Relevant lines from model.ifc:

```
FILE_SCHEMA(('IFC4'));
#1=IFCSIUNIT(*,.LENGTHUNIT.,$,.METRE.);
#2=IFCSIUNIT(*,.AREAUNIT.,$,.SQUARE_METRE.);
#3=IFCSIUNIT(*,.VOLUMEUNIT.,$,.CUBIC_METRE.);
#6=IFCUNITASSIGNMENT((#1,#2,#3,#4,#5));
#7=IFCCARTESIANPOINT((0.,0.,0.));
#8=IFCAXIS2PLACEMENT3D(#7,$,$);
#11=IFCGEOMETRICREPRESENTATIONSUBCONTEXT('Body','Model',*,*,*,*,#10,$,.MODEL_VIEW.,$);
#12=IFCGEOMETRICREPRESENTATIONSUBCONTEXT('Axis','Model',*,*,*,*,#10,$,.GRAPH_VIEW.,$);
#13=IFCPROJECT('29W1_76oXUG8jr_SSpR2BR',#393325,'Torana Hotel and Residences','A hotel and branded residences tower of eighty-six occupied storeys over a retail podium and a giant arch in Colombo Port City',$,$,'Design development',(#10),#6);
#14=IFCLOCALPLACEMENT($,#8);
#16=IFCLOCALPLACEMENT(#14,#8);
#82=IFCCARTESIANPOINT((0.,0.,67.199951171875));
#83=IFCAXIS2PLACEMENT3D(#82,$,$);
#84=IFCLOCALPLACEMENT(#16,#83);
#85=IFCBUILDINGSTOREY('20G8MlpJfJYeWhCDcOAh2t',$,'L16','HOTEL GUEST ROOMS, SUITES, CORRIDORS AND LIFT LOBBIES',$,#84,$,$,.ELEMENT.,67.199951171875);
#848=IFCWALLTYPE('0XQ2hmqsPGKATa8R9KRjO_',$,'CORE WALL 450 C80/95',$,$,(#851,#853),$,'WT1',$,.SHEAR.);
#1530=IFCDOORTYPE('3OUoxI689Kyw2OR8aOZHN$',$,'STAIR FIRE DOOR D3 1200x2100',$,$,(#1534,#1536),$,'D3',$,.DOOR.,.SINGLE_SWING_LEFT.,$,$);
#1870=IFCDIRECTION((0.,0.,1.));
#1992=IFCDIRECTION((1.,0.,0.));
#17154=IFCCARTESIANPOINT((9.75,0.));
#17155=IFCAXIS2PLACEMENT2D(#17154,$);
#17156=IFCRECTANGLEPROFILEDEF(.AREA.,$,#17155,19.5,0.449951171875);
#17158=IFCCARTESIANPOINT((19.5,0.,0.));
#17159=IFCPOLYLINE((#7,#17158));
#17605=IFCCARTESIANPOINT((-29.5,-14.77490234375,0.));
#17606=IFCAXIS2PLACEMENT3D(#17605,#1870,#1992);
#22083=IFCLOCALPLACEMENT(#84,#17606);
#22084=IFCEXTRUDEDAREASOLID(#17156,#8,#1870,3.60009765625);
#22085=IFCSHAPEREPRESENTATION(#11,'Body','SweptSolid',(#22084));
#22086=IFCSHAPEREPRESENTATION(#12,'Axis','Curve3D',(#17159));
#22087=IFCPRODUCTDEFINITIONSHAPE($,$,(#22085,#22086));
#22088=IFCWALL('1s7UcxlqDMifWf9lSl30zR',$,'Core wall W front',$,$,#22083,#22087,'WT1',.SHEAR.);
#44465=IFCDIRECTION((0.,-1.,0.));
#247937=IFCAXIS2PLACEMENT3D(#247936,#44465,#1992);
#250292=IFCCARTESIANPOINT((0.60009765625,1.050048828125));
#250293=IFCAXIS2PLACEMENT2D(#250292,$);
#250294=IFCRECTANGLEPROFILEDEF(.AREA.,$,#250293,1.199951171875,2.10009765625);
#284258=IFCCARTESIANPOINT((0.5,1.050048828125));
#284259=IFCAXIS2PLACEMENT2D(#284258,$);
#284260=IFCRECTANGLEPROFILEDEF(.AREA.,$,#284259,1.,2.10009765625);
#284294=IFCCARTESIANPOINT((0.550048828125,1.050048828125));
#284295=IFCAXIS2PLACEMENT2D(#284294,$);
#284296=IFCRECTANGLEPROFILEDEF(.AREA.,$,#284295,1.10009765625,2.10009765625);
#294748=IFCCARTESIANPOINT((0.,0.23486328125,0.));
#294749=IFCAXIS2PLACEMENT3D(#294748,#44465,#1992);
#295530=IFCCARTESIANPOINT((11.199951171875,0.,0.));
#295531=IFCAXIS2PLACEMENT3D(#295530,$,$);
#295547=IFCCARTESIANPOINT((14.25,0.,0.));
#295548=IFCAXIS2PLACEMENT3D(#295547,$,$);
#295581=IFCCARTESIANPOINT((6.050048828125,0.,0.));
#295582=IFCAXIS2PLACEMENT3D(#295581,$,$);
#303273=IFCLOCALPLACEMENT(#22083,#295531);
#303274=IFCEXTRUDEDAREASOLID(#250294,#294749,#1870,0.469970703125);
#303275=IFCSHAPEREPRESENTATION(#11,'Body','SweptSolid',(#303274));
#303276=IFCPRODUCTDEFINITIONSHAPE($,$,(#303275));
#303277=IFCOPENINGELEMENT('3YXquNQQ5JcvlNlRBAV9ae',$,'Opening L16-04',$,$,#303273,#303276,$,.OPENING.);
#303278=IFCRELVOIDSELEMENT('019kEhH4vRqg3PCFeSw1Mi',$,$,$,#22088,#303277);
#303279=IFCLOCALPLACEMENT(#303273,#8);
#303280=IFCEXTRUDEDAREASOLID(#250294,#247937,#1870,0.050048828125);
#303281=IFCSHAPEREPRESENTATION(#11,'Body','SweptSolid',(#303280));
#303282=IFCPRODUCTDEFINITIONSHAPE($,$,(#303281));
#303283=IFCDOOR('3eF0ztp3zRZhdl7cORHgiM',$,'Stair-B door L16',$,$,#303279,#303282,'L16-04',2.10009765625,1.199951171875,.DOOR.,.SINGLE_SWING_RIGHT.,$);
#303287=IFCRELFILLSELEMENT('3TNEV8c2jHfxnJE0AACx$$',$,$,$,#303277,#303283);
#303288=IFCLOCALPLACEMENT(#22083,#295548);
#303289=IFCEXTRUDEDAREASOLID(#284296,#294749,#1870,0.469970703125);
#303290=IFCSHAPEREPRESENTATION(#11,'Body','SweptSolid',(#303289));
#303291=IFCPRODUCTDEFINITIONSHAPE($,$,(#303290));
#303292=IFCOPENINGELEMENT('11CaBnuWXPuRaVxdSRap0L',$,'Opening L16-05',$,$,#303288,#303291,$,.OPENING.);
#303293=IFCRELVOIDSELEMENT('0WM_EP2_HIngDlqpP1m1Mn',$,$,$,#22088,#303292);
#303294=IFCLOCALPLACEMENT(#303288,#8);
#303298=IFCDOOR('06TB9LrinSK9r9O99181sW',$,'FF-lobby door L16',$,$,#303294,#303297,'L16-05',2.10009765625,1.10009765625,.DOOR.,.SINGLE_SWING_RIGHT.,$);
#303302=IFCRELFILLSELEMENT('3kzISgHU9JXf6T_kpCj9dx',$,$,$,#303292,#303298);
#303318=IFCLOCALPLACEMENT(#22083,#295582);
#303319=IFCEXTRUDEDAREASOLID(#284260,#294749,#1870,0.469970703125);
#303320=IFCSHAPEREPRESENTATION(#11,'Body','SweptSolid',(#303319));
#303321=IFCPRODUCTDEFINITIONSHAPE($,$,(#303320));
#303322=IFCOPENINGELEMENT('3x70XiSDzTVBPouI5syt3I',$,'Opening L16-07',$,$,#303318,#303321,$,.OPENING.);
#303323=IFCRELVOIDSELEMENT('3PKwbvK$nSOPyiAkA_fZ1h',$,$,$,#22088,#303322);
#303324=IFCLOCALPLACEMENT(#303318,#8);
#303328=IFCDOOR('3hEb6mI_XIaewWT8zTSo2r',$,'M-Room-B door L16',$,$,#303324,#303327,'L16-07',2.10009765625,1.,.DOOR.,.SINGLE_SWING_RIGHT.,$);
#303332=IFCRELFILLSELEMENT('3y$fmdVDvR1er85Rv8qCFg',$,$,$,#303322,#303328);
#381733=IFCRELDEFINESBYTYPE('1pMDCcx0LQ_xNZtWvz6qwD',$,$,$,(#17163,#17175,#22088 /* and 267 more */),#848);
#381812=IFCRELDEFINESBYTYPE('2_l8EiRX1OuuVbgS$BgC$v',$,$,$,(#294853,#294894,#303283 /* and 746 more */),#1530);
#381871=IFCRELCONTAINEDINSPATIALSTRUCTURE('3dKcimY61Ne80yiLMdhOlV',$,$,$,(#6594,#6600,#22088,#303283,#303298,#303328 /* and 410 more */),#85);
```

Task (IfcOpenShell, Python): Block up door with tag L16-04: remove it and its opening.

```python
import ifcopenshell
import ifcopenshell.api.feature
import ifcopenshell.api.root
import ifcopenshell.geom
import ifcopenshell.util.shape

model = ifcopenshell.open("model.ifc")
settings = ifcopenshell.geom.settings()


def volume(element):
    """Net volume in cubic metres, openings subtracted."""
    shape = ifcopenshell.geom.create_shape(settings, element)
    return ifcopenshell.util.shape.get_volume(shape.geometry)


door = model.by_guid("3eF0ztp3zRZhdl7cORHgiM")
opening = door.FillsVoids[0].RelatingOpeningElement
wall = opening.VoidsElements[0].RelatingBuildingElement
before = volume(wall)

ifcopenshell.api.root.remove_product(model, product=door)
ifcopenshell.api.feature.remove_feature(model, feature=opening)

after = volume(wall)

print(f"wall volume {before:.3f} -> {after:.3f} m3")

model.write("model_rev.ifc")
```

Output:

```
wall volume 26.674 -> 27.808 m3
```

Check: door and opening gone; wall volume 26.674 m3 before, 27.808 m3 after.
